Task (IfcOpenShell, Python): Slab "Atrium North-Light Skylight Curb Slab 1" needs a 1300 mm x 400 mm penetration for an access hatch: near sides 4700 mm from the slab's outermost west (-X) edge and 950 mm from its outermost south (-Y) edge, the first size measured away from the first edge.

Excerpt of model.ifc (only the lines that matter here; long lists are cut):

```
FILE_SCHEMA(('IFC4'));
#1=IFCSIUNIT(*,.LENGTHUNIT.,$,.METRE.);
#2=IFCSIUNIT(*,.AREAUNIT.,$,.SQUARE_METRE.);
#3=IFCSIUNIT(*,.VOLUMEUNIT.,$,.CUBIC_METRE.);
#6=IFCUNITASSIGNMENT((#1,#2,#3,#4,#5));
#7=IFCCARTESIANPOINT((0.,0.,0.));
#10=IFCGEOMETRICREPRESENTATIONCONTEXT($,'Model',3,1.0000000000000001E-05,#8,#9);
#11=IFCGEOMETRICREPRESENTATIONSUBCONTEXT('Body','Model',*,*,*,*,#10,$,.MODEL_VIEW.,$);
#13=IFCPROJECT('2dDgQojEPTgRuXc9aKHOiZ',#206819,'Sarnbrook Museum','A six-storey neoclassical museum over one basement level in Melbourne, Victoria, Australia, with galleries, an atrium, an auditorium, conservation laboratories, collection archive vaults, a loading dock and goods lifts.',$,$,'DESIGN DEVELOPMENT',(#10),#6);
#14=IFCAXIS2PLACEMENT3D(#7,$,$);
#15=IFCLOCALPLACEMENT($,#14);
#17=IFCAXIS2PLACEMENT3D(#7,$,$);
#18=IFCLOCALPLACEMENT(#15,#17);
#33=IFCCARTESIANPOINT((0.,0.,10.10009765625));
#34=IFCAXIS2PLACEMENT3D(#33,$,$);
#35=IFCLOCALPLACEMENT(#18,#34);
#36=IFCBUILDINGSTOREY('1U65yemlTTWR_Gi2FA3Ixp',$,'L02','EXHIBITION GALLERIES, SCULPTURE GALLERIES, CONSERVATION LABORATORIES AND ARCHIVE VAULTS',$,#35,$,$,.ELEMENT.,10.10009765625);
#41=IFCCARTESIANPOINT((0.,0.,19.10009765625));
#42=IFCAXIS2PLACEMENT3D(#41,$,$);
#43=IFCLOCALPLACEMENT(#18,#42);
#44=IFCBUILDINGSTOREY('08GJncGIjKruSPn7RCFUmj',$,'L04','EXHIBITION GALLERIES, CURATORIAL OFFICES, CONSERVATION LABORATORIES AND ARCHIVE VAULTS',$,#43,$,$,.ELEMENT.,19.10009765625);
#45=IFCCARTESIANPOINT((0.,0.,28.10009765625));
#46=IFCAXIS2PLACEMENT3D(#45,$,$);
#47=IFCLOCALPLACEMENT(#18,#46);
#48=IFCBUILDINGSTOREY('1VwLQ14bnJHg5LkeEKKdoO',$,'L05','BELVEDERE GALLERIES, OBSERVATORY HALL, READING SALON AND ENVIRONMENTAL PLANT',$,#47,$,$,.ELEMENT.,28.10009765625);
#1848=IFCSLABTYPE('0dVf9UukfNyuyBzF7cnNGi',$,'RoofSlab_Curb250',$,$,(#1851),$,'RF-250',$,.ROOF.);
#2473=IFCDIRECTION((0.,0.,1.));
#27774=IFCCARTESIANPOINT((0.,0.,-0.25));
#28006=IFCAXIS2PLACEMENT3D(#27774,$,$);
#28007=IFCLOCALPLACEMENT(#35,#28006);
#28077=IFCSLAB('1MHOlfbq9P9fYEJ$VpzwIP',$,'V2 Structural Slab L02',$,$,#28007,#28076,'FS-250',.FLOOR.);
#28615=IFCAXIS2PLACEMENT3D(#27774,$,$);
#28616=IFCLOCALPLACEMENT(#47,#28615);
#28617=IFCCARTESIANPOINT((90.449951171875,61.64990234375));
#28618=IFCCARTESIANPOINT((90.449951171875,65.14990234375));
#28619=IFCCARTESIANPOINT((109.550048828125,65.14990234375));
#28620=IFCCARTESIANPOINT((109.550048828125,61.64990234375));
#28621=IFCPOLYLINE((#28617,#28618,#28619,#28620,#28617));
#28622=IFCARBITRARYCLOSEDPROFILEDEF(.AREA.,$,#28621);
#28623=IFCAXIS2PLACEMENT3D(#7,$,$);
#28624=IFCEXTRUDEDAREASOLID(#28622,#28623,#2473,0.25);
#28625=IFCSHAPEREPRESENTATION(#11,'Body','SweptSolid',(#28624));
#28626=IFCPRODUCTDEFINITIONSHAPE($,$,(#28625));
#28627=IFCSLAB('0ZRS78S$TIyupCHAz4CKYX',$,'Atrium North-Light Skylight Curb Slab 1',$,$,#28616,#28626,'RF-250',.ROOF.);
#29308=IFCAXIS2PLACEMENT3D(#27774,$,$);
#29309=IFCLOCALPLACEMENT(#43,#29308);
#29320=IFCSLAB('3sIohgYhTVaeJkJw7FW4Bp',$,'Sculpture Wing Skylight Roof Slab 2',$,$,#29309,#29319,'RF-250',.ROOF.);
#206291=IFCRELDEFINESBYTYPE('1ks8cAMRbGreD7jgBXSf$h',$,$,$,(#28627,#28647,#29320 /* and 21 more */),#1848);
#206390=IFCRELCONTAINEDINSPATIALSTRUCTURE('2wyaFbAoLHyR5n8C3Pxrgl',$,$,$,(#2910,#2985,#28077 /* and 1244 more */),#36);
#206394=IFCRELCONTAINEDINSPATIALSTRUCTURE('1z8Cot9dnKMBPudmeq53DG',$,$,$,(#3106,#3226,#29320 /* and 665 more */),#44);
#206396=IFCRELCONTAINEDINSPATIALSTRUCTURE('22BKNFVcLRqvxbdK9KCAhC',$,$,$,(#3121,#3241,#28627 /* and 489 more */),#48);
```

```python
import numpy as np
import ifcopenshell
import ifcopenshell.api.feature
import ifcopenshell.api.geometry
import ifcopenshell.api.root
import ifcopenshell.geom
import ifcopenshell.util.placement
import ifcopenshell.util.representation
import ifcopenshell.util.shape
import ifcopenshell.util.unit

model = ifcopenshell.open("model.ifc")
unit_scale = ifcopenshell.util.unit.calculate_unit_scale(model)
settings = ifcopenshell.geom.settings()


def volume(element):
    """Net volume in cubic metres, openings subtracted."""
    shape = ifcopenshell.geom.create_shape(settings, element)
    return ifcopenshell.util.shape.get_volume(shape.geometry)


slab = model.by_guid("0ZRS78S$TIyupCHAz4CKYX")
before = volume(slab)

# Extent in the slab's own axes, in metres. The edges named are its -X and -Y sides.
slab_shape = ifcopenshell.geom.create_shape(settings, slab)
vertices = ifcopenshell.util.shape.get_vertices(slab_shape.geometry)
x_min, y_min, bottom = vertices.min(axis=0)
top = vertices[:, 2].max()

opening = ifcopenshell.api.root.create_entity(model, ifc_class="IfcOpeningElement", name="Access hatch opening", predefined_type="OPENING")
context = ifcopenshell.util.representation.get_context(model, "Model", "Body", "MODEL_VIEW")
width, depth = 1.3, 0.4
outline = [(0.0, 0.0), (width, 0.0), (width, depth), (0.0, depth), (0.0, 0.0)]
# Overshoot both faces by 50 mm so the cut is clean.
shape = ifcopenshell.api.geometry.add_slab_representation(
    model, context=context, depth=top - bottom + 0.1, polyline=outline
)
ifcopenshell.api.geometry.assign_representation(model, product=opening, representation=shape)

matrix = ifcopenshell.util.placement.get_local_placement(slab.ObjectPlacement)
matrix[:, 3] = matrix @ np.append(np.array([x_min + 4.7, y_min + 0.95, bottom - 0.05]) / unit_scale, 1.0)
ifcopenshell.api.geometry.edit_object_placement(model, product=opening, matrix=matrix, is_si=False)
ifcopenshell.api.feature.add_feature(model, feature=opening, element=slab)

after = volume(slab)

print(f"slab volume {before:.3f} -> {after:.3f} m3")

model.write("model_v2.ifc")
```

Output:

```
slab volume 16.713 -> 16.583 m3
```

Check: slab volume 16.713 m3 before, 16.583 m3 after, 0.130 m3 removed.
